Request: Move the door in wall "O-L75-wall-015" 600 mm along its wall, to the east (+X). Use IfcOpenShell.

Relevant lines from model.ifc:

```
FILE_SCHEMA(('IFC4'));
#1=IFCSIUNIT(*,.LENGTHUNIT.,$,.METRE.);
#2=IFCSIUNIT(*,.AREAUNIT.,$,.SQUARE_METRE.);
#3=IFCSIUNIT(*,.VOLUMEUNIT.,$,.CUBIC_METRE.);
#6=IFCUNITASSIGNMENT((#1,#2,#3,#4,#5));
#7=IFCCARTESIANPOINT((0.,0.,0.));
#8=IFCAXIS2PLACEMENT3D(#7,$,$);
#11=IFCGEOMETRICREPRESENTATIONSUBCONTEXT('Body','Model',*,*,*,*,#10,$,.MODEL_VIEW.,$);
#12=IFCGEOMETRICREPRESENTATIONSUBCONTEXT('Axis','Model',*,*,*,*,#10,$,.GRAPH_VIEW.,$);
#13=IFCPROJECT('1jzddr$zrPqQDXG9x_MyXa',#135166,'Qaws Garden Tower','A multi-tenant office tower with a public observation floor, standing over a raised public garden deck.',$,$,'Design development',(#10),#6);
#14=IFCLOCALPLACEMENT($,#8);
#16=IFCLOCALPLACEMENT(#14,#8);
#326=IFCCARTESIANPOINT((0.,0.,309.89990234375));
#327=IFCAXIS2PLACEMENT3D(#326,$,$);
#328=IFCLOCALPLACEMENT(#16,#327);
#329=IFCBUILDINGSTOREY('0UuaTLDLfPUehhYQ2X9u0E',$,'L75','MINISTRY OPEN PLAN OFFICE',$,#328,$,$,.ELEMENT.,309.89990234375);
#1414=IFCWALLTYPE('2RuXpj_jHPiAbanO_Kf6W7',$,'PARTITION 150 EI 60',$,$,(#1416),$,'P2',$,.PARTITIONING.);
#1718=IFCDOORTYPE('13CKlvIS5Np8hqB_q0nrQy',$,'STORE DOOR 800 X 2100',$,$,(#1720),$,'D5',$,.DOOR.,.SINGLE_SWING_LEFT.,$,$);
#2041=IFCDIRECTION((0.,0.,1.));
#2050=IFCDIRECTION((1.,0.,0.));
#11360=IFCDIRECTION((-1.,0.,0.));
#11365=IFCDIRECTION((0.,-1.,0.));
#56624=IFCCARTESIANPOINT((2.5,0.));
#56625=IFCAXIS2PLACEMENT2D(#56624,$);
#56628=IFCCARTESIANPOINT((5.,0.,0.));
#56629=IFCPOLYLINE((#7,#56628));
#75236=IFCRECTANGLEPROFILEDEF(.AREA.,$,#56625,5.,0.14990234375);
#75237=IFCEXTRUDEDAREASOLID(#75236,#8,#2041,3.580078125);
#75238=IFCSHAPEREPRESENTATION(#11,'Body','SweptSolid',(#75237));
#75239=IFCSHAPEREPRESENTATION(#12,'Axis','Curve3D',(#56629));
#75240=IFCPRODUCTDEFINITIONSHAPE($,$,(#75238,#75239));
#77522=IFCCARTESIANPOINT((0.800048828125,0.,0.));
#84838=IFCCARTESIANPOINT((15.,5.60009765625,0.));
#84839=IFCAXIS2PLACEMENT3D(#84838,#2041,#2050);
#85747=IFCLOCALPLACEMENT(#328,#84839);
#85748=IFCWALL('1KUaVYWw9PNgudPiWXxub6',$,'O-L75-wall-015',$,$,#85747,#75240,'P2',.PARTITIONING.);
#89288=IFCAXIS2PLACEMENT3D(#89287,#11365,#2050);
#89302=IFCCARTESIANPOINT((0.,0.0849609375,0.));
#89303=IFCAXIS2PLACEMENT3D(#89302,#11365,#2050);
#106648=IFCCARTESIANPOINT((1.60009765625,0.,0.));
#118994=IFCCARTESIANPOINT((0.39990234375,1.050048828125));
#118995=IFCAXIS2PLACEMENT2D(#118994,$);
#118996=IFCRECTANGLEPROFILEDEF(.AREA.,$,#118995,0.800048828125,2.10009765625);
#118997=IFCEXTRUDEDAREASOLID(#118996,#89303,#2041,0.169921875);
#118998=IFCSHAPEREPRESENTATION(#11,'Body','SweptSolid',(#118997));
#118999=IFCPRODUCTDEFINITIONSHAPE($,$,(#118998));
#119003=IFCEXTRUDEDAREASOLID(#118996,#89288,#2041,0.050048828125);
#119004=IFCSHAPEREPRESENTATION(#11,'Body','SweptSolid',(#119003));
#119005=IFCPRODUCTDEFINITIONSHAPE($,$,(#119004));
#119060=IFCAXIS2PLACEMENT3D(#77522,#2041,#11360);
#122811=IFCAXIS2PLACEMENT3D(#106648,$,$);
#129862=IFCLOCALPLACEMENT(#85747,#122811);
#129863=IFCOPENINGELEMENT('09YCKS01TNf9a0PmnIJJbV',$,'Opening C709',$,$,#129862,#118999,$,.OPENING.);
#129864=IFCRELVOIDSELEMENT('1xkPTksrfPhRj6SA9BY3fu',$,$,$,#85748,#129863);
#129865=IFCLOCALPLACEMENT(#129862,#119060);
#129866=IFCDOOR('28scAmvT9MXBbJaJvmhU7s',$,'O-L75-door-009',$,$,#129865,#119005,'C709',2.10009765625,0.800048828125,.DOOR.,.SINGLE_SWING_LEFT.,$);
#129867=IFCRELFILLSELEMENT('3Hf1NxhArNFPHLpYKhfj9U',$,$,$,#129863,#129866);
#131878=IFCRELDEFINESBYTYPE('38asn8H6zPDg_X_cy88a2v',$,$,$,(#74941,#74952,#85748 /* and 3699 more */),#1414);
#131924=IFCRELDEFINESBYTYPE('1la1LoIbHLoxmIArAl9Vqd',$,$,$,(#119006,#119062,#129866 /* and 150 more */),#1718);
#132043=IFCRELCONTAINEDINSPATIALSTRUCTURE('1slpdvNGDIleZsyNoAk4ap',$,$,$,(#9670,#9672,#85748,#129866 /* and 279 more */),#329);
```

```python
import ifcopenshell
import ifcopenshell.api.geometry
import ifcopenshell.util.placement

model = ifcopenshell.open("model.ifc")

door = model.by_id(129866)
opening = door.FillsVoids[0].RelatingOpeningElement
wall = opening.VoidsElements[0].RelatingBuildingElement

wall_matrix = ifcopenshell.util.placement.get_local_placement(wall.ObjectPlacement)
shift = wall_matrix[:3, 0] * 0.6
before = ifcopenshell.util.placement.get_local_placement(door.ObjectPlacement)[:3, 3].copy()

# The door is placed relative to its opening, so it follows when the opening moves.
matrix = ifcopenshell.util.placement.get_local_placement(opening.ObjectPlacement)
matrix[:3, 3] += shift
ifcopenshell.api.geometry.edit_object_placement(
    model, product=opening, matrix=matrix, is_si=False, should_transform_children=True
)

after = ifcopenshell.util.placement.get_local_placement(door.ObjectPlacement)[:3, 3]
print("door moved by", (after - before).round(3) + 0.0)

model.write("model_v2.ifc")
```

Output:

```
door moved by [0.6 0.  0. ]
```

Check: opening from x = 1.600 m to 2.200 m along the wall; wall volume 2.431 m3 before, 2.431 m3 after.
